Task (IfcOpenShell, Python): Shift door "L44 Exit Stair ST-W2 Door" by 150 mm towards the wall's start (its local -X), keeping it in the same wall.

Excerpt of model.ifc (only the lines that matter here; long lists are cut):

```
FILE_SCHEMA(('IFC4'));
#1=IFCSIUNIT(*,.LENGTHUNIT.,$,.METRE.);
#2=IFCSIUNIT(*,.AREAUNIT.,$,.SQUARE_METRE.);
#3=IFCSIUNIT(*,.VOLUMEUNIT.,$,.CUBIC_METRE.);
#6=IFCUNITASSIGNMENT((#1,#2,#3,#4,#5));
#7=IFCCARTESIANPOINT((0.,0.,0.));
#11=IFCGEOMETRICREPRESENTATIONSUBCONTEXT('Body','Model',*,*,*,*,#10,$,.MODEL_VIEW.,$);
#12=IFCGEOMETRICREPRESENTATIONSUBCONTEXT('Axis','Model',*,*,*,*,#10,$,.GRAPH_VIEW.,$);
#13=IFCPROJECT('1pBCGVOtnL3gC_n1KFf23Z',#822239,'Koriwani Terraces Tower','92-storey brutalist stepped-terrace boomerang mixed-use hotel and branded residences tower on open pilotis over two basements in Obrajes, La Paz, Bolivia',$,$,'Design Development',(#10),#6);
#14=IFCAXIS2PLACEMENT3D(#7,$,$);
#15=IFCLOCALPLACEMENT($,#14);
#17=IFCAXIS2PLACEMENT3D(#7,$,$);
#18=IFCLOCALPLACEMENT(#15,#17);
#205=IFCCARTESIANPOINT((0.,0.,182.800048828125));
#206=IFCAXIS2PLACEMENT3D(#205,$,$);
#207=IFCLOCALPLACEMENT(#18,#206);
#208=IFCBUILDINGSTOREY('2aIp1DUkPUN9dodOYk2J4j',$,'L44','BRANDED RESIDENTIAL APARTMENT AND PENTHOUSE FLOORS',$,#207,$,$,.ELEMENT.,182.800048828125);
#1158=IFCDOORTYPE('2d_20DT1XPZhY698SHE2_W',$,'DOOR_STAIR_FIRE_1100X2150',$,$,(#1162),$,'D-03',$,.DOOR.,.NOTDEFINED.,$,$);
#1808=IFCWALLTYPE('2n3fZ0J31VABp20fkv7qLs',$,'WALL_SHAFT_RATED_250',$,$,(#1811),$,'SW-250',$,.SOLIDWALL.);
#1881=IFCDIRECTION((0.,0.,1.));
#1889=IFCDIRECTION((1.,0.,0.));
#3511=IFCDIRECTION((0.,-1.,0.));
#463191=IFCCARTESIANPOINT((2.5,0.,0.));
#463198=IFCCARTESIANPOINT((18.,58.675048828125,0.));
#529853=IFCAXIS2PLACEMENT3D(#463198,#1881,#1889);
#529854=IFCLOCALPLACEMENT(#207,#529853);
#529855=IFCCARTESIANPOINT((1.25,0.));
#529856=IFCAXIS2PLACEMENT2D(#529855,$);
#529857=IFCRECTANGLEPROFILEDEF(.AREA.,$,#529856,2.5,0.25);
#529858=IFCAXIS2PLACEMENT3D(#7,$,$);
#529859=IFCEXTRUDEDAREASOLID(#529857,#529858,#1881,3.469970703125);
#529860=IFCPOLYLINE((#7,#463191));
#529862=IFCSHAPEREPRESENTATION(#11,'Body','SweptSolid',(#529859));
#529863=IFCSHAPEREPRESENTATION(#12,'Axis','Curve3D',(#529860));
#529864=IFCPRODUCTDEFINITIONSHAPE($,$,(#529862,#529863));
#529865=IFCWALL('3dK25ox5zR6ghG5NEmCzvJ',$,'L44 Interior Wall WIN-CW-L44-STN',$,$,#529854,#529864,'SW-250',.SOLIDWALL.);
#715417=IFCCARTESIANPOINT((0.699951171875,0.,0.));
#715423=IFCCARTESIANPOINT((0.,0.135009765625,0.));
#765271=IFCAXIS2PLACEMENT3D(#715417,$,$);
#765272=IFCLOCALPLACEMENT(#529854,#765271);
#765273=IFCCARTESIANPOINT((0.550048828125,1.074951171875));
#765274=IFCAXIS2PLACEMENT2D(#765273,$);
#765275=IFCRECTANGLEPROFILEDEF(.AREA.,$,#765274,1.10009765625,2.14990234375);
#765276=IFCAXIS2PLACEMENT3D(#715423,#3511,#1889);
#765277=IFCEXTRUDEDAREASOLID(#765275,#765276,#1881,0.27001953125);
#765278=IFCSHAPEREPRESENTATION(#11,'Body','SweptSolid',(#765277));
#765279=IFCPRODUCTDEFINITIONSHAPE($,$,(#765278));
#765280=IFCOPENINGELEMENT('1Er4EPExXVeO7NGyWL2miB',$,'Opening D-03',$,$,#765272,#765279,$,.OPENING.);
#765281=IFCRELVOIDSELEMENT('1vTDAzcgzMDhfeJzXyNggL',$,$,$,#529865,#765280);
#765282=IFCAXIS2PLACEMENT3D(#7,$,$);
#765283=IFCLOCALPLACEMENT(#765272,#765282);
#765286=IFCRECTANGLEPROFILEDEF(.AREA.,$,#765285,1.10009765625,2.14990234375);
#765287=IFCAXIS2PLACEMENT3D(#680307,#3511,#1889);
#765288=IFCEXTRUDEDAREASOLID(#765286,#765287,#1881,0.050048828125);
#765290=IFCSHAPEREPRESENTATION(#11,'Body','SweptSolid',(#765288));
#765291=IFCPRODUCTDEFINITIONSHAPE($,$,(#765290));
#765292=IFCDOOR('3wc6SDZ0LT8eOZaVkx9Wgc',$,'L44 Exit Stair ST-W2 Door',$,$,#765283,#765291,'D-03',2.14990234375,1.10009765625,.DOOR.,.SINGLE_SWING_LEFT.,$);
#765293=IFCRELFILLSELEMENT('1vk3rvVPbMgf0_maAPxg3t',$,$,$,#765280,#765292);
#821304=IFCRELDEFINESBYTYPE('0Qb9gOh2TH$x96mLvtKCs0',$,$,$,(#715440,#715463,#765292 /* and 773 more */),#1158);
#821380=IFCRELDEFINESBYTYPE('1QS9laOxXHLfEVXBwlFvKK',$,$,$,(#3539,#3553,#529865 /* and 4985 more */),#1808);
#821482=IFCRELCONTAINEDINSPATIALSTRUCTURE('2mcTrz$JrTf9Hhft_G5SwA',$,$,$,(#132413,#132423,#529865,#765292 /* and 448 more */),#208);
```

```python
import ifcopenshell
import ifcopenshell.api.geometry
import ifcopenshell.util.placement

model = ifcopenshell.open("model.ifc")

door = model.by_guid("3wc6SDZ0LT8eOZaVkx9Wgc")
opening = door.FillsVoids[0].RelatingOpeningElement
wall = opening.VoidsElements[0].RelatingBuildingElement

wall_matrix = ifcopenshell.util.placement.get_local_placement(wall.ObjectPlacement)
shift = wall_matrix[:3, 0] * -0.15
before = ifcopenshell.util.placement.get_local_placement(door.ObjectPlacement)[:3, 3].copy()

# The door is placed relative to its opening, so it follows when the opening moves.
matrix = ifcopenshell.util.placement.get_local_placement(opening.ObjectPlacement)
matrix[:3, 3] += shift
ifcopenshell.api.geometry.edit_object_placement(
    model, product=opening, matrix=matrix, is_si=False, should_transform_children=True
)

after = ifcopenshell.util.placement.get_local_placement(door.ObjectPlacement)[:3, 3]
print("door moved by", (after - before).round(3) + 0.0)

model.write("model_updated.ifc")
```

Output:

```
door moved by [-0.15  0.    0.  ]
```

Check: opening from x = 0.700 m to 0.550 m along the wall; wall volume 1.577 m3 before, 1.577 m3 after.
